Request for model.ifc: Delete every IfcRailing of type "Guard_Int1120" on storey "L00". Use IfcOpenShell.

First a look at what the model holds.

```python
import ifcopenshell
import ifcopenshell.util.element

model = ifcopenshell.open("model.ifc")
print(model.schema)
storey = next(s for s in model.by_type("IfcBuildingStorey") if s.Name == "L00")
railings = [e for e in ifcopenshell.util.element.get_decomposition(storey) if e.is_a("IfcRailing")]
seen = {}
for e in railings:
    element_type = ifcopenshell.util.element.get_type(e)
    name = element_type.Name if element_type not in (None, e) else None
    seen[name] = seen.get(name, 0) + 1
for name, count in sorted(seen.items(), key=str):
    print(count, "x", name)
```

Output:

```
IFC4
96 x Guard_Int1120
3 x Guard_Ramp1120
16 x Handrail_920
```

```python
import ifcopenshell
import ifcopenshell.api.root
import ifcopenshell.util.element

model = ifcopenshell.open("model.ifc")

storey = next(s for s in model.by_type("IfcBuildingStorey") if s.Name == "L00")
railings = [e for e in ifcopenshell.util.element.get_decomposition(storey) if e.is_a("IfcRailing")]
targets = [e for e in railings if (t := ifcopenshell.util.element.get_type(e)) not in (None, e) and t.Name == "Guard_Int1120"]

for e in targets:
    ifcopenshell.api.root.remove_product(model, product=e)
print(len(targets), "removed")

model.write("model_updated.ifc")
```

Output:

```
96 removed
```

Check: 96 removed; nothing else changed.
